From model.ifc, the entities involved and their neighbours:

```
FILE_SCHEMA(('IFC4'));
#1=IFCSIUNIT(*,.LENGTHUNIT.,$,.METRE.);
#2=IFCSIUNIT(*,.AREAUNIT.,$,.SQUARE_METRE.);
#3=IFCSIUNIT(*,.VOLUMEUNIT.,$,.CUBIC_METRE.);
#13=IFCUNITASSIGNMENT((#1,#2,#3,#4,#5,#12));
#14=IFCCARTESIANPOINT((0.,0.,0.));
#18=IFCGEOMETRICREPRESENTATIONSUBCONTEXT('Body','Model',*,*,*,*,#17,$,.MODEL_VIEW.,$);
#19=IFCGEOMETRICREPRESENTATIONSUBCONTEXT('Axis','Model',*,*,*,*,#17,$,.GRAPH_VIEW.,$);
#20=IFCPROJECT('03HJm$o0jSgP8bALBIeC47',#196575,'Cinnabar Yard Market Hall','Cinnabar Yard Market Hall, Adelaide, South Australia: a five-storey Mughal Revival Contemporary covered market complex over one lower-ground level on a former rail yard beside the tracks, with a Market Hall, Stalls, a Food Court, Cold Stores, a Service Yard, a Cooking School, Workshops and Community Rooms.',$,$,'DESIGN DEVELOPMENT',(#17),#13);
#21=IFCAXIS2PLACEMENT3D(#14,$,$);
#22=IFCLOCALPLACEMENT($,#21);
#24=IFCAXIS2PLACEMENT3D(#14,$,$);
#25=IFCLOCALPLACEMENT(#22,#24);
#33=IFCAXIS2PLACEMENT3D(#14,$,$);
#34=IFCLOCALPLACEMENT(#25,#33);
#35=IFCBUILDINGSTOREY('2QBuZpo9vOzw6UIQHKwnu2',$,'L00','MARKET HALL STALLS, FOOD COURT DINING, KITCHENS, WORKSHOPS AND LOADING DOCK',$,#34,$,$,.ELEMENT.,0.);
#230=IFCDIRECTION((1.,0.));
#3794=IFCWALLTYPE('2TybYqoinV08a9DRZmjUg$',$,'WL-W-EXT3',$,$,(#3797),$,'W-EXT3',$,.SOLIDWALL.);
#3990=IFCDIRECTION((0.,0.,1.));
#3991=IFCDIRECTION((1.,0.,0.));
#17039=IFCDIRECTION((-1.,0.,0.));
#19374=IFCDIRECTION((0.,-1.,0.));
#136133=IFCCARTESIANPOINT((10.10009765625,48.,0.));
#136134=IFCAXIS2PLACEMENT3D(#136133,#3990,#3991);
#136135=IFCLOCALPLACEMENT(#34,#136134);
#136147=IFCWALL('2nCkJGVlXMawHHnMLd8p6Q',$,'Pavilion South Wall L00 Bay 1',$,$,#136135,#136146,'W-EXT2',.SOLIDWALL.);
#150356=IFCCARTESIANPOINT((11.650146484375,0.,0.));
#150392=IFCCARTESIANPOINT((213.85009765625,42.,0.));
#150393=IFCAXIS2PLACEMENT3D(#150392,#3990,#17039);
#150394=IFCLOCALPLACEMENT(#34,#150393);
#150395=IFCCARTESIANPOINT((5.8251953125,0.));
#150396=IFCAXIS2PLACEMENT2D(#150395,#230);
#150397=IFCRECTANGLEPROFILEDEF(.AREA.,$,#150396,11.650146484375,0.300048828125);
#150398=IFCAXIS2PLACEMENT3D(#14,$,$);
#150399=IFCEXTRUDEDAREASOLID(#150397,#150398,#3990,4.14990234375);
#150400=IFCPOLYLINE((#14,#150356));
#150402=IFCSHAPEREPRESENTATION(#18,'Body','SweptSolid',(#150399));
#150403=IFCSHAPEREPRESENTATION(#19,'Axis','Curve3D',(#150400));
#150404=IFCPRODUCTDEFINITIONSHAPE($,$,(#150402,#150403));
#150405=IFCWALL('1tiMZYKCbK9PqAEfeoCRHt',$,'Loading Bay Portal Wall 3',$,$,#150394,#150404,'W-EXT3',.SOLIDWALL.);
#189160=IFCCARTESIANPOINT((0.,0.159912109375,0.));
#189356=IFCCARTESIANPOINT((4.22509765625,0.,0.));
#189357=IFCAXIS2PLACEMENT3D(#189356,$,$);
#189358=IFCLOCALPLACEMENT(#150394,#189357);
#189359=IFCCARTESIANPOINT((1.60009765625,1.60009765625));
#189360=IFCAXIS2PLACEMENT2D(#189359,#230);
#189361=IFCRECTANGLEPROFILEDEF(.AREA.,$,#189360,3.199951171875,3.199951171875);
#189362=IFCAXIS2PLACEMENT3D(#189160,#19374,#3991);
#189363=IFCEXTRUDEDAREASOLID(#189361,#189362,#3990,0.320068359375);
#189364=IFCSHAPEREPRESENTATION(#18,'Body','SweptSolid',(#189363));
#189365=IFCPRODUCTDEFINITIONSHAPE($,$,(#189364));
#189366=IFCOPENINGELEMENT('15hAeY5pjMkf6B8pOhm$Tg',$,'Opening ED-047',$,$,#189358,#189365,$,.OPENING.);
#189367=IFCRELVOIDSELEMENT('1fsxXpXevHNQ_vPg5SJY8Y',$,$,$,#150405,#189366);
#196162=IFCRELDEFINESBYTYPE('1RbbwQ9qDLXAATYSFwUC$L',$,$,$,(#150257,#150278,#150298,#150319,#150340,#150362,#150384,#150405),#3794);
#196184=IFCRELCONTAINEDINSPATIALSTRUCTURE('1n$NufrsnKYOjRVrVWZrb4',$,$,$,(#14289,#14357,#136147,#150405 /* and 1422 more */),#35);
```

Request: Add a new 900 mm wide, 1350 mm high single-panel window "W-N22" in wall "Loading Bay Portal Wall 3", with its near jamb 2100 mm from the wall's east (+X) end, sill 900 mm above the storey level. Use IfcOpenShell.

```python
import numpy as np
import ifcopenshell
import ifcopenshell.api.feature
import ifcopenshell.api.geometry
import ifcopenshell.api.root
import ifcopenshell.api.spatial
import ifcopenshell.geom
import ifcopenshell.util.element
import ifcopenshell.util.placement
import ifcopenshell.util.representation
import ifcopenshell.util.shape
import ifcopenshell.util.unit

model = ifcopenshell.open("model.ifc")
unit_scale = ifcopenshell.util.unit.calculate_unit_scale(model)
settings = ifcopenshell.geom.settings()


def volume(element):
    """Net volume in cubic metres, openings subtracted."""
    shape = ifcopenshell.geom.create_shape(settings, element)
    return ifcopenshell.util.shape.get_volume(shape.geometry)


wall = model.by_guid("1tiMZYKCbK9PqAEfeoCRHt")
storey = ifcopenshell.util.element.get_container(wall, ifc_class="IfcBuildingStorey")
context = ifcopenshell.util.representation.get_context(model, "Model", "Body", "MODEL_VIEW")
before = volume(wall)

width, height, from_end, sill = 0.9, 1.35, 2.1, 0.9  # metres

# The wall runs along its own X axis, and the end named is its -X end.
wall_shape = ifcopenshell.geom.create_shape(settings, wall)
x, y, z = ifcopenshell.util.shape.get_vertices(wall_shape.geometry).T
start = x.min() + from_end
face, thickness = float(y.min()), float(y.max() - y.min())
wall_matrix = ifcopenshell.util.placement.get_local_placement(wall.ObjectPlacement)
level = ifcopenshell.util.placement.get_local_placement(storey.ObjectPlacement)[2, 3]


def in_wall(x, y):
    """Placement at x, y metres in the wall's axes, at sill height."""
    matrix = wall_matrix.copy()
    matrix[:, 3] = wall_matrix @ np.array([x / unit_scale, y / unit_scale, 0.0, 1.0])
    matrix[2, 3] = level + sill / unit_scale
    return matrix


# Opening: a box that overshoots both wall faces by 50 mm.
opening = ifcopenshell.api.root.create_entity(model, ifc_class="IfcOpeningElement", predefined_type="OPENING")
box = ifcopenshell.api.geometry.add_wall_representation(
    model, context=context, length=width, height=height, thickness=thickness + 0.1
)
ifcopenshell.api.geometry.assign_representation(model, product=opening, representation=box)
ifcopenshell.api.geometry.edit_object_placement(model, product=opening, matrix=in_wall(start, face - 0.05), is_si=False)
ifcopenshell.api.feature.add_feature(model, feature=opening, element=wall)

window = ifcopenshell.api.root.create_entity(model, ifc_class="IfcWindow", name="W-N22", predefined_type="WINDOW")
window.OverallWidth, window.OverallHeight = width / unit_scale, height / unit_scale
window.PartitioningType = "SINGLE_PANEL"
body = ifcopenshell.api.geometry.add_window_representation(
    model,
    context=context,
    overall_width=window.OverallWidth,
    overall_height=window.OverallHeight,
    partition_type="SINGLE_PANEL",
)
ifcopenshell.api.geometry.assign_representation(model, product=window, representation=body)
ifcopenshell.api.spatial.assign_container(model, products=[window], relating_structure=storey)
ifcopenshell.api.feature.add_filling(model, opening=opening, element=window)

# Centre the window in the wall's thickness.
ifcopenshell.api.geometry.edit_object_placement(model, product=window, matrix=in_wall(start, face), is_si=False)
window_shape = ifcopenshell.geom.create_shape(settings, window)
depth = ifcopenshell.util.shape.get_vertices(window_shape.geometry)[:, 1]
offset = face + thickness / 2 - (depth.min() + depth.max()) / 2
ifcopenshell.api.geometry.edit_object_placement(model, product=window, matrix=in_wall(start, offset), is_si=False)

after = volume(wall)

print(f"wall volume {before:.3f} -> {after:.3f} m3")

model.write("model_updated.ifc")
```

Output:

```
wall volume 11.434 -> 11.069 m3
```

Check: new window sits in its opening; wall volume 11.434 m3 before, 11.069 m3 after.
